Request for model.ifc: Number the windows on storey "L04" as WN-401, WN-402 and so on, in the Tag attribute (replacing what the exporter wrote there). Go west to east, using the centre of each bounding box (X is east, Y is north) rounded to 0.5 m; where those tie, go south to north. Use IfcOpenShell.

First a look at what the model holds.

```python
import ifcopenshell
import ifcopenshell.util.element
import ifcopenshell.util.placement

model = ifcopenshell.open("model.ifc")
print(model.schema)
storey = next(s for s in model.by_type("IfcBuildingStorey") if s.Name == "L04")
windows = [e for e in ifcopenshell.util.element.get_decomposition(storey) if e.is_a("IfcWindow")]
for e in sorted(windows, key=lambda e: e.id()):
    origin = ifcopenshell.util.placement.get_local_placement(e.ObjectPlacement)[:3, 3]
    print(e.id(), e.Tag, e.Name, origin.round(2) + 0.0, sep=" | ")
```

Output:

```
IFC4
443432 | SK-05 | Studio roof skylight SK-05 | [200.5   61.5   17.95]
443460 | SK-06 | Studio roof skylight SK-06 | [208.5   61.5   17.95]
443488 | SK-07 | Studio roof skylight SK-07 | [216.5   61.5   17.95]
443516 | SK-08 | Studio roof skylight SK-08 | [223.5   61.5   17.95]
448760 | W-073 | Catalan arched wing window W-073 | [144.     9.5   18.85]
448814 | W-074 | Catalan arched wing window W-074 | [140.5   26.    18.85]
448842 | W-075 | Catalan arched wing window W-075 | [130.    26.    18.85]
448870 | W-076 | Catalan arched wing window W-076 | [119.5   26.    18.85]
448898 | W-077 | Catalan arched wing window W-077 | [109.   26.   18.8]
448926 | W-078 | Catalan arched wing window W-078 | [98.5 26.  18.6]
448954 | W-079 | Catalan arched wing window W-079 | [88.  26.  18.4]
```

```python
import ifcopenshell
import ifcopenshell.geom
import ifcopenshell.util.element
import ifcopenshell.util.shape

model = ifcopenshell.open("model.ifc")
settings = ifcopenshell.geom.settings()
settings.set("use-world-coords", True)


def centre(element):
    shape = ifcopenshell.geom.create_shape(settings, element)
    return ifcopenshell.util.shape.get_bbox_centroid(shape.geometry)


storey = next(s for s in model.by_type("IfcBuildingStorey") if s.Name == "L04")
windows = [e for e in ifcopenshell.util.element.get_decomposition(storey) if e.is_a("IfcWindow")]

# Insertion points can sit at a corner or the storey origin, so sort by the geometry (in metres).
centres = {e: centre(e) for e in windows}
windows.sort(key=lambda e: (round(centres[e][0] / 0.5), centres[e][1]))

for i, e in enumerate(windows, start=1):
    number = f"WN-4{i:02d}"
    e.Tag = number
    print(e.id(), number)

model.write("model_updated.ifc")
```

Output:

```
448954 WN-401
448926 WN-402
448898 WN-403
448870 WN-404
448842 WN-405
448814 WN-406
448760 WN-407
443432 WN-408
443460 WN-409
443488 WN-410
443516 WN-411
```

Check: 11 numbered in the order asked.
